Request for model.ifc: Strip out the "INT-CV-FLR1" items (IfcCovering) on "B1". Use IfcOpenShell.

First a look at what the model holds.

```python
import ifcopenshell
import ifcopenshell.util.element

model = ifcopenshell.open("model.ifc")
print(model.schema)
storey = next(s for s in model.by_type("IfcBuildingStorey") if s.Name == "B1")
coverings = [e for e in ifcopenshell.util.element.get_decomposition(storey) if e.is_a("IfcCovering")]
seen = {}
for e in coverings:
    element_type = ifcopenshell.util.element.get_type(e)
    name = element_type.Name if element_type not in (None, e) else None
    seen[name] = seen.get(name, 0) + 1
for name, count in sorted(seen.items(), key=str):
    print(count, "x", name)
```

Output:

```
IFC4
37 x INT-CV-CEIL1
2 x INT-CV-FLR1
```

```python
import ifcopenshell
import ifcopenshell.api.root
import ifcopenshell.util.element

model = ifcopenshell.open("model.ifc")

storey = next(s for s in model.by_type("IfcBuildingStorey") if s.Name == "B1")
coverings = [e for e in ifcopenshell.util.element.get_decomposition(storey) if e.is_a("IfcCovering")]
targets = [e for e in coverings if (t := ifcopenshell.util.element.get_type(e)) not in (None, e) and t.Name == "INT-CV-FLR1"]

for e in targets:
    ifcopenshell.api.root.remove_product(model, product=e)
print(len(targets), "removed")

model.write("model_v2.ifc")
```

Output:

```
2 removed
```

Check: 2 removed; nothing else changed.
